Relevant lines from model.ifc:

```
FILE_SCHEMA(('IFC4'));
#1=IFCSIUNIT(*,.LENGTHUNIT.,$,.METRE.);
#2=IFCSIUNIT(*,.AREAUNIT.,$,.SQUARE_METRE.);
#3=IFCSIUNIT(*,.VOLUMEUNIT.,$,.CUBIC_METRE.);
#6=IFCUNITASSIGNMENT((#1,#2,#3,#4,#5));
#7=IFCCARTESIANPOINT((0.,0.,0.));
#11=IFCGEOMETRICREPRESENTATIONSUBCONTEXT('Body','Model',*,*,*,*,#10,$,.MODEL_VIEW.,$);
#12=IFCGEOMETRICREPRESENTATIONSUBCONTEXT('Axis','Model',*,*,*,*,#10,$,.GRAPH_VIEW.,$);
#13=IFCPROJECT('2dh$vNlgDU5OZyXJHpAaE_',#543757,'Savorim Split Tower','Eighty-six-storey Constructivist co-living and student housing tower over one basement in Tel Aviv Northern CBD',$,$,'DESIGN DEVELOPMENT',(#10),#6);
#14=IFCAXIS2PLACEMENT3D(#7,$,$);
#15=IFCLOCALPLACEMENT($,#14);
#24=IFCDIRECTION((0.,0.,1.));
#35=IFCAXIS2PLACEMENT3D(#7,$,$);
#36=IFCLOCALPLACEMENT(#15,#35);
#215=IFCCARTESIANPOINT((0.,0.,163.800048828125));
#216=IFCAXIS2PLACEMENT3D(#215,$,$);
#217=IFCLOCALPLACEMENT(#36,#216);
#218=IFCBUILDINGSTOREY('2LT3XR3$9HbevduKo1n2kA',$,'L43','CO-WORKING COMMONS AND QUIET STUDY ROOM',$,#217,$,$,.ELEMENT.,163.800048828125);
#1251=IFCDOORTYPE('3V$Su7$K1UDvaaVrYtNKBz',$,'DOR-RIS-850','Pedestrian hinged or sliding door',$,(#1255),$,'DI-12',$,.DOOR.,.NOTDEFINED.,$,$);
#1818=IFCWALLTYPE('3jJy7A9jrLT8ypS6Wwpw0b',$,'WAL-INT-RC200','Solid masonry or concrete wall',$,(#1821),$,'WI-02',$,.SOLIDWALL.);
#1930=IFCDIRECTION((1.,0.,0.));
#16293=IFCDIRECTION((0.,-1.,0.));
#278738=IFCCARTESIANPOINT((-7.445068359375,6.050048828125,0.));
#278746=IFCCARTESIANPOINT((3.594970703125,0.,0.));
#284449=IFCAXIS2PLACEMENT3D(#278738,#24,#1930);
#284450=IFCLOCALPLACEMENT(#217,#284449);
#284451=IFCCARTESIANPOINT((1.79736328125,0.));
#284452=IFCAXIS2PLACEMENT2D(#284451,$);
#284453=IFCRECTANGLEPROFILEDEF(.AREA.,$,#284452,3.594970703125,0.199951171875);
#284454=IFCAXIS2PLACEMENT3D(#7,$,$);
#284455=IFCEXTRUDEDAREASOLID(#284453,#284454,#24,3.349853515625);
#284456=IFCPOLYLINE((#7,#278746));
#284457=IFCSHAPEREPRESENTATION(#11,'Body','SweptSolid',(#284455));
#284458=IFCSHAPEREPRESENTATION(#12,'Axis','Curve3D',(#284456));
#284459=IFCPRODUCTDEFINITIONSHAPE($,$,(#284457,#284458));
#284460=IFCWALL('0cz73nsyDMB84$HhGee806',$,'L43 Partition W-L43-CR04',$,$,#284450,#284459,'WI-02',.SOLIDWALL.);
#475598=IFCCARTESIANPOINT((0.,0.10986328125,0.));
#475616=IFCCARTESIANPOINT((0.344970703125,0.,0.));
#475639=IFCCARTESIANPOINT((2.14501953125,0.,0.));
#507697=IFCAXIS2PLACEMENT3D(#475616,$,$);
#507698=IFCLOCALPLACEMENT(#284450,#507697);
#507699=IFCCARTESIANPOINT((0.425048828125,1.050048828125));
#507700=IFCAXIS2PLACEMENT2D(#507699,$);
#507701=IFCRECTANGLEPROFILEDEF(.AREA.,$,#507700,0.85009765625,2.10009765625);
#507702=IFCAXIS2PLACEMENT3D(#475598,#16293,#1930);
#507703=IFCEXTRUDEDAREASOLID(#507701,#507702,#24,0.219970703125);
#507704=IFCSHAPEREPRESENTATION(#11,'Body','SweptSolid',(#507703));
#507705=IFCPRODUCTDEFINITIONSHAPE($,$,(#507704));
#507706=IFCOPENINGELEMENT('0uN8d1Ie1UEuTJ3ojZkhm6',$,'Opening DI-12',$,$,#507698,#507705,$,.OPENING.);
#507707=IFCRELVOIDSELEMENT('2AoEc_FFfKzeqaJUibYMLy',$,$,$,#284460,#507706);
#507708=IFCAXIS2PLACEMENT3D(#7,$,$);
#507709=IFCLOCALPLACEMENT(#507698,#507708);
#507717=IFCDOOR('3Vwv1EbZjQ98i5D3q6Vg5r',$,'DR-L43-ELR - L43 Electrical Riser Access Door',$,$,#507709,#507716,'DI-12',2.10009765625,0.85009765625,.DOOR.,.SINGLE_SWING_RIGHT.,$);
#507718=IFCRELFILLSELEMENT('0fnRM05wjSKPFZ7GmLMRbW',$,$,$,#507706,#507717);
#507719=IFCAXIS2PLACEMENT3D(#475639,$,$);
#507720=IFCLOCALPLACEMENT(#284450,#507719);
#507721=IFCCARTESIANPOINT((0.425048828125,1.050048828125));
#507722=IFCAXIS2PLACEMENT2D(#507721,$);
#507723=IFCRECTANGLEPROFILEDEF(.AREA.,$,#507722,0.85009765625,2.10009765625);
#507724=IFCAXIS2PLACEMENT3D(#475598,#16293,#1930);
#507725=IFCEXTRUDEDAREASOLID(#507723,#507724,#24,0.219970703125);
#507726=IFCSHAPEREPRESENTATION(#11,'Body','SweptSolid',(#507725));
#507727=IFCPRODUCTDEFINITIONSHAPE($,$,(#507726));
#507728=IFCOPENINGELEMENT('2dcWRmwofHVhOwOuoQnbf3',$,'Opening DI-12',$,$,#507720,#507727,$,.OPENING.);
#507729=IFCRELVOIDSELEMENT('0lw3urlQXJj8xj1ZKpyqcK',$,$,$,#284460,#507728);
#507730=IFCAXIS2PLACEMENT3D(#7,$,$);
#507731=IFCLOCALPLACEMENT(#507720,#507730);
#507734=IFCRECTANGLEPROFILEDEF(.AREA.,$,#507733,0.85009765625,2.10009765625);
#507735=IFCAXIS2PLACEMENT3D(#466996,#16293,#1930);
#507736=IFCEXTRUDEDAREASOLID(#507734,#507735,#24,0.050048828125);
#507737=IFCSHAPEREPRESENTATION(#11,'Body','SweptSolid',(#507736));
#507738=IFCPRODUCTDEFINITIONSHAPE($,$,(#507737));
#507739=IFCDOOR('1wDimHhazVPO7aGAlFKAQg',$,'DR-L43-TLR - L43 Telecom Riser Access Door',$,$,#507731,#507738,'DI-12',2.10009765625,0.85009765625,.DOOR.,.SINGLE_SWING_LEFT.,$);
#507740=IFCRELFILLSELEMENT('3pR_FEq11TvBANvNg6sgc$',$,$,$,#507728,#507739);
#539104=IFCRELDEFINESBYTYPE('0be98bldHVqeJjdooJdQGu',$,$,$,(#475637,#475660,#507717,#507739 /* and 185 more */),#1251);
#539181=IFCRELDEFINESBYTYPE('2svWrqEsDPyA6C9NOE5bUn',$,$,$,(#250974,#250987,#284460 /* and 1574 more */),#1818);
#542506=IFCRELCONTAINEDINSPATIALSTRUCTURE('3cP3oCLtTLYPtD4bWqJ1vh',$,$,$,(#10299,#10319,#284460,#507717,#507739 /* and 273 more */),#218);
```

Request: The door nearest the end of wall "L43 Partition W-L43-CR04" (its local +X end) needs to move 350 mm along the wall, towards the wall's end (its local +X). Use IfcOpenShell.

```python
import ifcopenshell
import ifcopenshell.api.geometry
import ifcopenshell.util.placement
import ifcopenshell.util.unit

model = ifcopenshell.open("model.ifc")
unit_scale = ifcopenshell.util.unit.calculate_unit_scale(model)

door = model.by_id(507739)
opening = door.FillsVoids[0].RelatingOpeningElement
wall = opening.VoidsElements[0].RelatingBuildingElement

wall_matrix = ifcopenshell.util.placement.get_local_placement(wall.ObjectPlacement)
shift = wall_matrix[:3, 0] * 0.35 / unit_scale
before = ifcopenshell.util.placement.get_local_placement(door.ObjectPlacement)[:3, 3].copy()

# The door is placed relative to its opening, so it follows when the opening moves.
matrix = ifcopenshell.util.placement.get_local_placement(opening.ObjectPlacement)
matrix[:3, 3] += shift
ifcopenshell.api.geometry.edit_object_placement(
    model, product=opening, matrix=matrix, is_si=False, should_transform_children=True
)

after = ifcopenshell.util.placement.get_local_placement(door.ObjectPlacement)[:3, 3]
print("door moved by", (after - before).round(3) + 0.0)

model.write("model_rev.ifc")
```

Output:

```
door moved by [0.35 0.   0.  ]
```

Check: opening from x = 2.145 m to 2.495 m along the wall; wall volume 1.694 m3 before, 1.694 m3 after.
